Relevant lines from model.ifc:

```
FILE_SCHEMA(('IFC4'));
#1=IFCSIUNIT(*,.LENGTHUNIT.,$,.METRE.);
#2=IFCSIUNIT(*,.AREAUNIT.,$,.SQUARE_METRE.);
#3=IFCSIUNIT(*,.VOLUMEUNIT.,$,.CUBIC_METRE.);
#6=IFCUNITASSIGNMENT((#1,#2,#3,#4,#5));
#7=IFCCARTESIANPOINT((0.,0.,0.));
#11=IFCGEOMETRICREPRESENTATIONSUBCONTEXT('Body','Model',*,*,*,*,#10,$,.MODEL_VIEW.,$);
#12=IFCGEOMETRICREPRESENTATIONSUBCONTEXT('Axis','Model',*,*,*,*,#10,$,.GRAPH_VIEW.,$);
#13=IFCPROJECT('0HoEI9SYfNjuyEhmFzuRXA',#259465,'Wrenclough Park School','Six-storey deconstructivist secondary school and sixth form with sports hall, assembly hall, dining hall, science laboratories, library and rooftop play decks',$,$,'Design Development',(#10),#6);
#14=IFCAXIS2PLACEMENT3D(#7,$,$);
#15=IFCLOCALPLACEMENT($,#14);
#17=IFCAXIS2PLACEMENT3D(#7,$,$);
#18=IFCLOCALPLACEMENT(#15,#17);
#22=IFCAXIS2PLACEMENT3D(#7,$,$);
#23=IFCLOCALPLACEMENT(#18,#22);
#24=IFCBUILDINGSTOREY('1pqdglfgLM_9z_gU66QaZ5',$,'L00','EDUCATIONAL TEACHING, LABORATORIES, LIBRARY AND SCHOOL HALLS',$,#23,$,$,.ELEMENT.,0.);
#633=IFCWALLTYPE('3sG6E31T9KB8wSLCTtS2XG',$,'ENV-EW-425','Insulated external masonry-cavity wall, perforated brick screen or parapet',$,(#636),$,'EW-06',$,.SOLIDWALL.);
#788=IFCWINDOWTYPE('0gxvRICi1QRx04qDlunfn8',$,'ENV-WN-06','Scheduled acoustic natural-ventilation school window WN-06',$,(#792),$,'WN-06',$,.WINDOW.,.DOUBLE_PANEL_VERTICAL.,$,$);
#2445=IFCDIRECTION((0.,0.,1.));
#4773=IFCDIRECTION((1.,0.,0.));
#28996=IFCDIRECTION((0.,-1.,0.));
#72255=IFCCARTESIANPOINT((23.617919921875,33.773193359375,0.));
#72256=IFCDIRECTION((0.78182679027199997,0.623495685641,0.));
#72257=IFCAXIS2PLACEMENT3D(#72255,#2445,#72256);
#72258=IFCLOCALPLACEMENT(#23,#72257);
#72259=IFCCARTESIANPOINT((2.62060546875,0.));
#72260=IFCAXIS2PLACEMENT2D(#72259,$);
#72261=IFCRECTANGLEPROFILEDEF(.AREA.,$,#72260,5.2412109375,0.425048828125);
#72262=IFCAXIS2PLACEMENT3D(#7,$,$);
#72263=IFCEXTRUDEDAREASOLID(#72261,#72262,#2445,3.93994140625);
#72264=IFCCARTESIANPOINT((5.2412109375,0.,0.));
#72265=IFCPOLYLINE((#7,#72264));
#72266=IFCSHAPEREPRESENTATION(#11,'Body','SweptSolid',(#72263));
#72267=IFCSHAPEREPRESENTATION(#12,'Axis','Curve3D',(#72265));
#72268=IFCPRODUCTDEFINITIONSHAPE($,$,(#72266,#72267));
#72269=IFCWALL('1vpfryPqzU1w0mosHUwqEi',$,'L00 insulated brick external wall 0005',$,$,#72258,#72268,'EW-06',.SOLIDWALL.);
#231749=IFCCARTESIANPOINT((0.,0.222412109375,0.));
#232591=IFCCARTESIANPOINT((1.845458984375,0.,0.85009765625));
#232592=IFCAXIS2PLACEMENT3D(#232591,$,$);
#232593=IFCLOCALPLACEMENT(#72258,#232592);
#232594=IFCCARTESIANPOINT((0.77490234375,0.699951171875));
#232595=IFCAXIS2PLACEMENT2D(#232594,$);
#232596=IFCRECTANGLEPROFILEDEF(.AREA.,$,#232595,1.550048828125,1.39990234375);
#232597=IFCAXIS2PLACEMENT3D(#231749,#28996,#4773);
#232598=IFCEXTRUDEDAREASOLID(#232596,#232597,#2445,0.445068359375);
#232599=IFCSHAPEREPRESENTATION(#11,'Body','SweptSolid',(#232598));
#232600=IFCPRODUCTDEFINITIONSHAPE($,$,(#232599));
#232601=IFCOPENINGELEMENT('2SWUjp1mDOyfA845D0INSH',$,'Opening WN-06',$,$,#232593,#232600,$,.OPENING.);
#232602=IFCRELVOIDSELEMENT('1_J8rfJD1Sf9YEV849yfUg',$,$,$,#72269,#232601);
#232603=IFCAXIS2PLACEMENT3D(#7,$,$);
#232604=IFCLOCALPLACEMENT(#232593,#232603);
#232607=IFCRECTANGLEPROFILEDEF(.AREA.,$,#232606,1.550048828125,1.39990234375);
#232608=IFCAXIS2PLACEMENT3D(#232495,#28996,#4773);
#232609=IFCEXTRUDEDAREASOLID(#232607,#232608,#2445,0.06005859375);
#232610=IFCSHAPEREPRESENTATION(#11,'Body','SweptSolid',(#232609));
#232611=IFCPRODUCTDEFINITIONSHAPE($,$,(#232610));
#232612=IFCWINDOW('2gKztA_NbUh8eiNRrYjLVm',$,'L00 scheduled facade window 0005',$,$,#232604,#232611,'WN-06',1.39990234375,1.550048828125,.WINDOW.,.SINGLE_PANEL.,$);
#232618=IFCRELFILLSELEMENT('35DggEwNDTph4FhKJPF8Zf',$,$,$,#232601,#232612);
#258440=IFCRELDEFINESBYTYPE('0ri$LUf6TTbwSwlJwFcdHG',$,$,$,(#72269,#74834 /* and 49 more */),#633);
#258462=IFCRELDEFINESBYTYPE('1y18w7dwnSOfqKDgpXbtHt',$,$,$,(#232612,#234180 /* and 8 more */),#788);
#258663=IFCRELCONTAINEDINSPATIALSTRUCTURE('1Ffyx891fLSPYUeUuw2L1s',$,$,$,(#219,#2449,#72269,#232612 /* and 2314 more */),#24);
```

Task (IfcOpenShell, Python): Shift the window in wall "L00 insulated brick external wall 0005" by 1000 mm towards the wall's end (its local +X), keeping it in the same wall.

```python
import ifcopenshell
import ifcopenshell.api.geometry
import ifcopenshell.util.placement
import ifcopenshell.util.unit

model = ifcopenshell.open("model.ifc")
unit_scale = ifcopenshell.util.unit.calculate_unit_scale(model)

window = model.by_id(232612)
opening = window.FillsVoids[0].RelatingOpeningElement
wall = opening.VoidsElements[0].RelatingBuildingElement

wall_matrix = ifcopenshell.util.placement.get_local_placement(wall.ObjectPlacement)
shift = wall_matrix[:3, 0] * 1 / unit_scale
before = ifcopenshell.util.placement.get_local_placement(window.ObjectPlacement)[:3, 3].copy()

# The window is placed relative to its opening, so it follows when the opening moves.
matrix = ifcopenshell.util.placement.get_local_placement(opening.ObjectPlacement)
matrix[:3, 3] += shift
ifcopenshell.api.geometry.edit_object_placement(
    model, product=opening, matrix=matrix, is_si=False, should_transform_children=True
)

after = ifcopenshell.util.placement.get_local_placement(window.ObjectPlacement)[:3, 3]
print("window moved by", (after - before).round(3) + 0.0)

model.write("model_updated.ifc")
```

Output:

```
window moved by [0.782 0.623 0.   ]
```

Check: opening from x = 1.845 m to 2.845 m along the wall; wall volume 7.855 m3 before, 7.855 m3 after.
